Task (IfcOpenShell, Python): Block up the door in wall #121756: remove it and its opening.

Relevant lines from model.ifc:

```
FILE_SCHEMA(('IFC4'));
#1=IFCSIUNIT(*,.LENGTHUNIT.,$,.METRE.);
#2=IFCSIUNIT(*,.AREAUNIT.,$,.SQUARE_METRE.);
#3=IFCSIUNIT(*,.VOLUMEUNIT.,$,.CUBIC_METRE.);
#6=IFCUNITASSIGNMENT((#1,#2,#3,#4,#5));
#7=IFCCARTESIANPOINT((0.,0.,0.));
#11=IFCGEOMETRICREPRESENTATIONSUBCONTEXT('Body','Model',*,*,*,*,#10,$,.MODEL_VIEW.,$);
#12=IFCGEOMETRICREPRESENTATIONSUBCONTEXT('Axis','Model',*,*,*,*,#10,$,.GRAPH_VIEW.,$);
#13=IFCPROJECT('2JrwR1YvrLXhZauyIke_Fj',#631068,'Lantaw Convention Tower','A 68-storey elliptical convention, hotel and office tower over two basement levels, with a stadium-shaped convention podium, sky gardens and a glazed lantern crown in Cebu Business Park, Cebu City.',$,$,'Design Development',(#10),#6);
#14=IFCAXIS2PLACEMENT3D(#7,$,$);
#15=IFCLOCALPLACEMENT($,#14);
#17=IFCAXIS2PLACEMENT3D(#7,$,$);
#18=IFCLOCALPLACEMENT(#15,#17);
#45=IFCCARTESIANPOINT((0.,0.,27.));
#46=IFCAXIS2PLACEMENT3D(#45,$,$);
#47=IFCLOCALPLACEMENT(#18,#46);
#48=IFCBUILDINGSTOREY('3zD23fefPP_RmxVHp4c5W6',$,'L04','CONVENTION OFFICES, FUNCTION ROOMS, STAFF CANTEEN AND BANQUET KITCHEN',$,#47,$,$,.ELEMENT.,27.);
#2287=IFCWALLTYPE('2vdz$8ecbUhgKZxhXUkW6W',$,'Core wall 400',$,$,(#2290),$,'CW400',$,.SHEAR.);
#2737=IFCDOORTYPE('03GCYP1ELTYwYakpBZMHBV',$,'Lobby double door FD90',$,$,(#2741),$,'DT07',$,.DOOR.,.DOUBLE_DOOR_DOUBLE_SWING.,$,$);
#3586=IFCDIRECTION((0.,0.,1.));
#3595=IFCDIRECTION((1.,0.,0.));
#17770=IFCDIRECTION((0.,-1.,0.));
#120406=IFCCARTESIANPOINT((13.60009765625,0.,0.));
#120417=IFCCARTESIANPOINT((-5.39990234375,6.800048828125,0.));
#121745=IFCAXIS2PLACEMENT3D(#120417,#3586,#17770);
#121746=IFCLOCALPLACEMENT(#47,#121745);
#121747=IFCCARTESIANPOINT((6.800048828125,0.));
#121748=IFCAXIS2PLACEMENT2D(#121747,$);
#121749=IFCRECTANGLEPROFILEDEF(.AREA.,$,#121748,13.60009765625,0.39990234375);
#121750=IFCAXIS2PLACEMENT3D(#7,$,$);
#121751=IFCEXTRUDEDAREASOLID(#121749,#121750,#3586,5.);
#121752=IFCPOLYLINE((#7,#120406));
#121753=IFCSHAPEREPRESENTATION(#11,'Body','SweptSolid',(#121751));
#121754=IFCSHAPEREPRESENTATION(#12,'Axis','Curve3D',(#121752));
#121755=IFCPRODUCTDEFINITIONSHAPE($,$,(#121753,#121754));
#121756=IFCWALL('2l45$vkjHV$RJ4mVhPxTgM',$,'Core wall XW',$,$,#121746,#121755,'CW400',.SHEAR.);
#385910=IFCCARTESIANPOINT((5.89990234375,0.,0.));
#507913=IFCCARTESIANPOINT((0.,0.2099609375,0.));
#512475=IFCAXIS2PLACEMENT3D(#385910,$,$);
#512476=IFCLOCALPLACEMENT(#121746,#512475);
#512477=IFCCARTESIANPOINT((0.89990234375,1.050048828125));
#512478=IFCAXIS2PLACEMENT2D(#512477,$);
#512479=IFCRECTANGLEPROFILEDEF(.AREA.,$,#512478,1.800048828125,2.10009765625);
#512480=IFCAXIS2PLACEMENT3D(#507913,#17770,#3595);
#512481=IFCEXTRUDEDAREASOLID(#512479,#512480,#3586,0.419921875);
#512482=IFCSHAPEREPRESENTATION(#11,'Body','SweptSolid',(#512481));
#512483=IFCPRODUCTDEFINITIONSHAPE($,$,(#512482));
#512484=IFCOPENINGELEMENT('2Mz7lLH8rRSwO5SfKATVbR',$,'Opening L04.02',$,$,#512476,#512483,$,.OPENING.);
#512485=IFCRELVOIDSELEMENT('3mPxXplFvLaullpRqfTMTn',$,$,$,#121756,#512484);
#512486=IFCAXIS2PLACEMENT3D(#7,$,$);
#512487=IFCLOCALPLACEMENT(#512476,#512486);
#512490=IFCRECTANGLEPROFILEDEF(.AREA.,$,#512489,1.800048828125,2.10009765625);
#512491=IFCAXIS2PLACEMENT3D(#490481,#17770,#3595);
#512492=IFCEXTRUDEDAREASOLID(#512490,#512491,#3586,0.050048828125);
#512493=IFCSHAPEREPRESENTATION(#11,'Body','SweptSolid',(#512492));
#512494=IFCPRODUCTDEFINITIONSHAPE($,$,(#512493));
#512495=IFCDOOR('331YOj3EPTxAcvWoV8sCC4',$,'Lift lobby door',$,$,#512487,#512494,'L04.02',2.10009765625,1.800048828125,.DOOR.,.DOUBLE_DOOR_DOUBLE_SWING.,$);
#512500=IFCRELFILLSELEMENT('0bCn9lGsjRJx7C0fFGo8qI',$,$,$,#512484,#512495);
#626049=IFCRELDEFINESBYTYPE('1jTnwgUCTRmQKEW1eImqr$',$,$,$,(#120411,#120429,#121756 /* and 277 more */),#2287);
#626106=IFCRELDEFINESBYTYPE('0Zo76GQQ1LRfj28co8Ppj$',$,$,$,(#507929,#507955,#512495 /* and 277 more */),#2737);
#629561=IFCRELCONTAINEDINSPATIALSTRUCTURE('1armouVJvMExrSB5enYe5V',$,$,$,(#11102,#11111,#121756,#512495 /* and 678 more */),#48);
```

```python
import ifcopenshell
import ifcopenshell.api.feature
import ifcopenshell.api.root
import ifcopenshell.geom
import ifcopenshell.util.shape

model = ifcopenshell.open("model.ifc")
settings = ifcopenshell.geom.settings()


def volume(element):
    """Net volume in cubic metres, openings subtracted."""
    shape = ifcopenshell.geom.create_shape(settings, element)
    return ifcopenshell.util.shape.get_volume(shape.geometry)


door = model.by_guid("331YOj3EPTxAcvWoV8sCC4")
opening = door.FillsVoids[0].RelatingOpeningElement
wall = opening.VoidsElements[0].RelatingBuildingElement
before = volume(wall)

ifcopenshell.api.root.remove_product(model, product=door)
ifcopenshell.api.feature.remove_feature(model, feature=opening)

after = volume(wall)

print(f"wall volume {before:.3f} -> {after:.3f} m3")

model.write("model_rev.ifc")
```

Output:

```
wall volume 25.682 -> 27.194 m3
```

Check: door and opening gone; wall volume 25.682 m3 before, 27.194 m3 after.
